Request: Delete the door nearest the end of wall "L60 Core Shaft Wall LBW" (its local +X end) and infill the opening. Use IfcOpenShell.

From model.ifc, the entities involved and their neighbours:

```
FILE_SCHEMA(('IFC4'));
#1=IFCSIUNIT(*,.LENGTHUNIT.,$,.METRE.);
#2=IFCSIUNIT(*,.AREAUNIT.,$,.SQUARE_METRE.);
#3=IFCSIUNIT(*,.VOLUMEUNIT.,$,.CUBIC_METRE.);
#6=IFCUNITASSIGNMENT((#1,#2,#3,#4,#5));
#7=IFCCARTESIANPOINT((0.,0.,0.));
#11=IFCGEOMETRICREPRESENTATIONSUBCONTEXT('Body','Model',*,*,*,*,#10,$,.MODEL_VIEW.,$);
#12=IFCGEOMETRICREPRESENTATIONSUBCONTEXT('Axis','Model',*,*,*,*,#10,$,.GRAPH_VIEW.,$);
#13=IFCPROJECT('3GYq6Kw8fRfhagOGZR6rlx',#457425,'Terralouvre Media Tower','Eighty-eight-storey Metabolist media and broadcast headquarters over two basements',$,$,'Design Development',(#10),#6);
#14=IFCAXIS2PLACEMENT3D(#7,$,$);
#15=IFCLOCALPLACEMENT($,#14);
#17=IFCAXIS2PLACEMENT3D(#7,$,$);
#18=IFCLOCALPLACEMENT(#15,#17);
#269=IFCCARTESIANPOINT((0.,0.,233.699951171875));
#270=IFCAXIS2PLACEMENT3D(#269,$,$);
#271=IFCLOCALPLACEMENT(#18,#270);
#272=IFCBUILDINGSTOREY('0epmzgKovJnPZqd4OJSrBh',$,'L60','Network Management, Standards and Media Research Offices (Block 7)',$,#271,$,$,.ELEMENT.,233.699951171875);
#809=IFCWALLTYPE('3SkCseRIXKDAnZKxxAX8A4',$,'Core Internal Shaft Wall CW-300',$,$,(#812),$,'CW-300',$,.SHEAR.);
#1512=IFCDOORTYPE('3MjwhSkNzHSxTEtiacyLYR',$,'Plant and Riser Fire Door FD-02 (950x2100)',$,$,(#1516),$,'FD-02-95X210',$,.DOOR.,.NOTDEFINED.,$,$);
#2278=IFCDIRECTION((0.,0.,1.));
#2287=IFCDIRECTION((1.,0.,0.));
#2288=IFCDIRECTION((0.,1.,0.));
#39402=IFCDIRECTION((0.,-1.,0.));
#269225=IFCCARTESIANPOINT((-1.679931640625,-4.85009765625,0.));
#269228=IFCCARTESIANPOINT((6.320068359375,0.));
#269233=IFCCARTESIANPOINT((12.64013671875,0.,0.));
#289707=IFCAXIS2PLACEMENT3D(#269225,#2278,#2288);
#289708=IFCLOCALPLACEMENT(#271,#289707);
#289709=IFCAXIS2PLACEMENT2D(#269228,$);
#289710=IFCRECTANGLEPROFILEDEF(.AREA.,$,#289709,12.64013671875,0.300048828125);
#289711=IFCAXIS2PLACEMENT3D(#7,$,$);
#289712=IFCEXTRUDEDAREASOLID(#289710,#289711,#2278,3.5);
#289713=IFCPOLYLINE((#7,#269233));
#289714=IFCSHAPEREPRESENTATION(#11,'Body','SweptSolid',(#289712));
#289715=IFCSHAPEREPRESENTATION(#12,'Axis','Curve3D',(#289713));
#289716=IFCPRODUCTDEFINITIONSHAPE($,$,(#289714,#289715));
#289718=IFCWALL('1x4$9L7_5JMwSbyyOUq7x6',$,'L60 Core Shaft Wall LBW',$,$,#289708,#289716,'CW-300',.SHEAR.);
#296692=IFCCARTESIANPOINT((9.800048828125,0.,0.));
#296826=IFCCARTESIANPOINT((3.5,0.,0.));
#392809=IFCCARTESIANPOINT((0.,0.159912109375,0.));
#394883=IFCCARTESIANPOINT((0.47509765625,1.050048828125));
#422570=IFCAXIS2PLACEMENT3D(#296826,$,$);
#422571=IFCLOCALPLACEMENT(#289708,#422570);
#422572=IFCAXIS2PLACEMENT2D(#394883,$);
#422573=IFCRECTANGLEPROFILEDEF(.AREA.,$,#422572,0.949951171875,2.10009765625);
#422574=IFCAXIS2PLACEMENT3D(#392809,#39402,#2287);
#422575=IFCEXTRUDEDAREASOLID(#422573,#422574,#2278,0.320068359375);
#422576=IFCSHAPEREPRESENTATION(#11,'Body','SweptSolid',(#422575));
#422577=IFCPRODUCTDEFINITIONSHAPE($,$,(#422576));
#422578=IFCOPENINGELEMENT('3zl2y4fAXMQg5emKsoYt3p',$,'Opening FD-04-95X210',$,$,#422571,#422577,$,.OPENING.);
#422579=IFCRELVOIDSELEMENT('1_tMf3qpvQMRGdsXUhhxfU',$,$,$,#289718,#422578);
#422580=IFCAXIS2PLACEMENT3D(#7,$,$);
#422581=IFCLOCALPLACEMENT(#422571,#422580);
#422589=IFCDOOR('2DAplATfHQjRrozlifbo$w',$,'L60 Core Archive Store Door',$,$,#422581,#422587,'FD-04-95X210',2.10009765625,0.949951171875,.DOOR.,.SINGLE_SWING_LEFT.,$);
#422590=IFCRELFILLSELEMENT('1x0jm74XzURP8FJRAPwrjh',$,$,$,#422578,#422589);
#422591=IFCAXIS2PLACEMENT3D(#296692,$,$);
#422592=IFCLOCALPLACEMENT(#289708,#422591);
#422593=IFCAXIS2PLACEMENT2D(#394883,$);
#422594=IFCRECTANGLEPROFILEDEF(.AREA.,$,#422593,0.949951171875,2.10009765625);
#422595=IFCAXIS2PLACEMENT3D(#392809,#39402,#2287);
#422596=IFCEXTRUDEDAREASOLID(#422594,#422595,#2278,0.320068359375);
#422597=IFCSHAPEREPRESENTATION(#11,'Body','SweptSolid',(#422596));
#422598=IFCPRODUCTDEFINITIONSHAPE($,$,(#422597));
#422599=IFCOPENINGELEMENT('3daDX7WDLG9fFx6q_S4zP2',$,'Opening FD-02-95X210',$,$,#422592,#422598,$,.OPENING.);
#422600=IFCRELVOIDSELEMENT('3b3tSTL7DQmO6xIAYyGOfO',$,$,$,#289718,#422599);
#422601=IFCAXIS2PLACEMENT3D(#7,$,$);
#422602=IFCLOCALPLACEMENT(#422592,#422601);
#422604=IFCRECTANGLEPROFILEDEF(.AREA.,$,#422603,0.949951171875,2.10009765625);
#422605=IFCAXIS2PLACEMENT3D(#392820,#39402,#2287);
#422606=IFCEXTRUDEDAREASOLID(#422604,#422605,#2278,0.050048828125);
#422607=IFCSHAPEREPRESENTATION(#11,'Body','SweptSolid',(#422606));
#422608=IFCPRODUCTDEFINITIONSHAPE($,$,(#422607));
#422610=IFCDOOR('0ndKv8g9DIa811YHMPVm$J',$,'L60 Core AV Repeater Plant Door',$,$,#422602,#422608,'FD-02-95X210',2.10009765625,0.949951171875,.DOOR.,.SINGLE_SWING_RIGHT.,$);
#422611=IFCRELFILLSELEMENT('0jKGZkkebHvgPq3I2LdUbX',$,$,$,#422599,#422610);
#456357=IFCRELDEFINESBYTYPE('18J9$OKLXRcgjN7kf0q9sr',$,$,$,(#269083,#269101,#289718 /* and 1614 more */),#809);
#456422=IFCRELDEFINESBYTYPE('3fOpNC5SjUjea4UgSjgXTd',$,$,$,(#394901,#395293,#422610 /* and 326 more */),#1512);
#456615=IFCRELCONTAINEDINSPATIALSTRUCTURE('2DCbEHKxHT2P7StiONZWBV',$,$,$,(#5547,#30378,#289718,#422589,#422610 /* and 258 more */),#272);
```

```python
import ifcopenshell
import ifcopenshell.api.feature
import ifcopenshell.api.root
import ifcopenshell.geom
import ifcopenshell.util.shape

model = ifcopenshell.open("model.ifc")
settings = ifcopenshell.geom.settings()


def volume(element):
    """Net volume in cubic metres, openings subtracted."""
    shape = ifcopenshell.geom.create_shape(settings, element)
    return ifcopenshell.util.shape.get_volume(shape.geometry)


door = model.by_guid("0ndKv8g9DIa811YHMPVm$J")
opening = door.FillsVoids[0].RelatingOpeningElement
wall = opening.VoidsElements[0].RelatingBuildingElement
before = volume(wall)

ifcopenshell.api.root.remove_product(model, product=door)
ifcopenshell.api.feature.remove_feature(model, feature=opening)

after = volume(wall)

print(f"wall volume {before:.3f} -> {after:.3f} m3")

model.write("model_v2.ifc")
```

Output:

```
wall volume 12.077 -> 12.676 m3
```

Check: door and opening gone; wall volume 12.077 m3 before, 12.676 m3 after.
